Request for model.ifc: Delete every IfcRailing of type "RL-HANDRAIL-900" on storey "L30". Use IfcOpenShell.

First a look at what the model holds.

```python
import ifcopenshell
import ifcopenshell.util.element

model = ifcopenshell.open("model.ifc")
print(model.schema)
storey = next(s for s in model.by_type("IfcBuildingStorey") if s.Name == "L30")
railings = [e for e in ifcopenshell.util.element.get_decomposition(storey) if e.is_a("IfcRailing")]
seen = {}
for e in railings:
    element_type = ifcopenshell.util.element.get_type(e)
    name = element_type.Name if element_type not in (None, e) else None
    seen[name] = seen.get(name, 0) + 1
for name, count in sorted(seen.items(), key=str):
    print(count, "x", name)
```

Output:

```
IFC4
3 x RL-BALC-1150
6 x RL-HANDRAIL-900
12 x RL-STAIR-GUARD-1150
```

```python
import ifcopenshell
import ifcopenshell.api.root
import ifcopenshell.util.element

model = ifcopenshell.open("model.ifc")

storey = next(s for s in model.by_type("IfcBuildingStorey") if s.Name == "L30")
railings = [e for e in ifcopenshell.util.element.get_decomposition(storey) if e.is_a("IfcRailing")]
targets = [e for e in railings if (t := ifcopenshell.util.element.get_type(e)) not in (None, e) and t.Name == "RL-HANDRAIL-900"]

for e in targets:
    ifcopenshell.api.root.remove_product(model, product=e)
print(len(targets), "removed")

model.write("model-out.ifc")
```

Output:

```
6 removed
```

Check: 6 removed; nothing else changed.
